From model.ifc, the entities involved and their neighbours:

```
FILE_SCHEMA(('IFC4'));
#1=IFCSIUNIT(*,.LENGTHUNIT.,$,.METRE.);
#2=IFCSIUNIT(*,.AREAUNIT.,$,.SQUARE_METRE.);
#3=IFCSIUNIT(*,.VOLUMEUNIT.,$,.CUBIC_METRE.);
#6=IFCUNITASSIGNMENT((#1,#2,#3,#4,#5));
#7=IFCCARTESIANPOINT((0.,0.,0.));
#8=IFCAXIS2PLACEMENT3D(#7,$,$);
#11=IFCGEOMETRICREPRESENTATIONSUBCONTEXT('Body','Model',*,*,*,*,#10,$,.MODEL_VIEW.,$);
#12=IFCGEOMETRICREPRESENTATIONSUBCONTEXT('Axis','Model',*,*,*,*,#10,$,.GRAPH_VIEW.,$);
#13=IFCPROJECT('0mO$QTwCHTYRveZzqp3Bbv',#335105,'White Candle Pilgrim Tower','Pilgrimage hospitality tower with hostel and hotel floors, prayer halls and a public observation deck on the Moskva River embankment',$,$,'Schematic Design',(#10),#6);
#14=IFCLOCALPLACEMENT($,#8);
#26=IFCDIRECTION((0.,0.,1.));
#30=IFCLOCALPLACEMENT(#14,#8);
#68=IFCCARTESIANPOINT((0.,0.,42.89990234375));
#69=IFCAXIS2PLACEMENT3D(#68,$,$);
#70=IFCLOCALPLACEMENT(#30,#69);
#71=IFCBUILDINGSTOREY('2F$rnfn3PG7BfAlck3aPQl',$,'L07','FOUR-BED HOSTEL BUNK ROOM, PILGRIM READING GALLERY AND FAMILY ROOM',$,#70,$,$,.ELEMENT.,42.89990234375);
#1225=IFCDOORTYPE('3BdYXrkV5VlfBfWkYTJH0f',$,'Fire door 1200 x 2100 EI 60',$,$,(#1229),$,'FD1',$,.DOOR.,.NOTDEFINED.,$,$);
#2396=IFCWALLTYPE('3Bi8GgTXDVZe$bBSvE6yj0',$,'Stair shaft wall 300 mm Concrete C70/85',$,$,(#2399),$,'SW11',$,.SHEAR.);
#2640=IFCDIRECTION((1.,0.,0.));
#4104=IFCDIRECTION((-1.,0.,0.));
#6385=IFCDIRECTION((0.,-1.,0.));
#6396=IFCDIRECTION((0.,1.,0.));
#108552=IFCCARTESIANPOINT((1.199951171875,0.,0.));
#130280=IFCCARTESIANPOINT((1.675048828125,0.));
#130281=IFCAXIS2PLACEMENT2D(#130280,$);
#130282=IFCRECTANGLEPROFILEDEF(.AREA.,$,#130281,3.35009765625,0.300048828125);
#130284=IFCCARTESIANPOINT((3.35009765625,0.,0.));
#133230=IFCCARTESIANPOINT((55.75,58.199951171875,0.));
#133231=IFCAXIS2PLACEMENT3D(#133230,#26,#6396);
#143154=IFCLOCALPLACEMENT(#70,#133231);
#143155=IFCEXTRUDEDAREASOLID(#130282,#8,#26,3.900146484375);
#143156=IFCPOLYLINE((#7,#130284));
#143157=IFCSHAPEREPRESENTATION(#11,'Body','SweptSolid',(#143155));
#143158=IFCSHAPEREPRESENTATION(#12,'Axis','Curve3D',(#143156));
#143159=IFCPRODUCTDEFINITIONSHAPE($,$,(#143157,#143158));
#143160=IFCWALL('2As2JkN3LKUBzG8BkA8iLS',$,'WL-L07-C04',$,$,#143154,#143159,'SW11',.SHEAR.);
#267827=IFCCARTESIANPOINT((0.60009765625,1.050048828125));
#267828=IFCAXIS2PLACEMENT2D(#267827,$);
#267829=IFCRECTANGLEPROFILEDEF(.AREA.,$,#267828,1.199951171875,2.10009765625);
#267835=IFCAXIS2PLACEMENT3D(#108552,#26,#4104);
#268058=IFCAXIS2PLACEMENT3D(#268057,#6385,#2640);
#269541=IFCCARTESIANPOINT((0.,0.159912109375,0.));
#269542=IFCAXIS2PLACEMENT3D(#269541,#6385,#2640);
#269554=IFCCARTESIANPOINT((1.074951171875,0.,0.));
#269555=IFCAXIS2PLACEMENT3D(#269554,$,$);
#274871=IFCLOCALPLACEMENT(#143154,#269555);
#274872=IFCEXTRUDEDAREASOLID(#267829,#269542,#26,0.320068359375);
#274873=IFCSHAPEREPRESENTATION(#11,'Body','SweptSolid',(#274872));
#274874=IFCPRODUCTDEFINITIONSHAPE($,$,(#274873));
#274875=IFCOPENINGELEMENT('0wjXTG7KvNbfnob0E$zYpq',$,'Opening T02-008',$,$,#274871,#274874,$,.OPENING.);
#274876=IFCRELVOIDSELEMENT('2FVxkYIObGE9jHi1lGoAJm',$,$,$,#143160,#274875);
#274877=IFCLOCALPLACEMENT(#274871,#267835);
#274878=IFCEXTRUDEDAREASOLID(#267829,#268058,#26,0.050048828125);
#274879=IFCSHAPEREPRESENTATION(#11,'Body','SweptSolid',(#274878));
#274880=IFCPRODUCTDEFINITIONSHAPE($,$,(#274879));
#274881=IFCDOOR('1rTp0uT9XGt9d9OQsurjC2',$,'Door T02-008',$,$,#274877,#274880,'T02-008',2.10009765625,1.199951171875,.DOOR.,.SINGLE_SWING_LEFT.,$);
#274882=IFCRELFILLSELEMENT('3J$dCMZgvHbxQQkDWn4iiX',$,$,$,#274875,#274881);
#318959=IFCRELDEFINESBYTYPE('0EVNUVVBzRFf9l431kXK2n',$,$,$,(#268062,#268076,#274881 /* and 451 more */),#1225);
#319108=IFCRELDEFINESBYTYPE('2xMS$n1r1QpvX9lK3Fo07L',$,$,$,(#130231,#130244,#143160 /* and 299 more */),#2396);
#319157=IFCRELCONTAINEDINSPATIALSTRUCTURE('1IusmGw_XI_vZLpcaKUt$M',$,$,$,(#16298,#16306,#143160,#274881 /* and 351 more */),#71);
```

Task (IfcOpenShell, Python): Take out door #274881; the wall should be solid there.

```python
import ifcopenshell
import ifcopenshell.api.feature
import ifcopenshell.api.root
import ifcopenshell.geom
import ifcopenshell.util.shape

model = ifcopenshell.open("model.ifc")
settings = ifcopenshell.geom.settings()


def volume(element):
    """Net volume in cubic metres, openings subtracted."""
    shape = ifcopenshell.geom.create_shape(settings, element)
    return ifcopenshell.util.shape.get_volume(shape.geometry)


door = model.by_guid("1rTp0uT9XGt9d9OQsurjC2")
opening = door.FillsVoids[0].RelatingOpeningElement
wall = opening.VoidsElements[0].RelatingBuildingElement
before = volume(wall)

ifcopenshell.api.root.remove_product(model, product=door)
ifcopenshell.api.feature.remove_feature(model, feature=opening)

after = volume(wall)

print(f"wall volume {before:.3f} -> {after:.3f} m3")

model.write("model_v2.ifc")
```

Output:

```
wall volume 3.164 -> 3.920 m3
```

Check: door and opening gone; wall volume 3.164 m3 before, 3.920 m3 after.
